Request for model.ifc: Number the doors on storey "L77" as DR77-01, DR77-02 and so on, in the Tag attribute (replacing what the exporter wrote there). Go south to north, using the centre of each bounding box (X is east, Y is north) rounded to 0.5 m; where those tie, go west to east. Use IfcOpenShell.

First a look at what the model holds.

```python
import ifcopenshell
import ifcopenshell.util.element
import ifcopenshell.util.placement

model = ifcopenshell.open("model.ifc")
print(model.schema)
storey = next(s for s in model.by_type("IfcBuildingStorey") if s.Name == "L77")
doors = [e for e in ifcopenshell.util.element.get_decomposition(storey) if e.is_a("IfcDoor")]
for e in sorted(doors, key=lambda e: e.id()):
    origin = ifcopenshell.util.placement.get_local_placement(e.ObjectPlacement)[:3, 3]
    print(e.id(), e.Tag, e.Name, origin.round(2) + 0.0, sep=" | ")
```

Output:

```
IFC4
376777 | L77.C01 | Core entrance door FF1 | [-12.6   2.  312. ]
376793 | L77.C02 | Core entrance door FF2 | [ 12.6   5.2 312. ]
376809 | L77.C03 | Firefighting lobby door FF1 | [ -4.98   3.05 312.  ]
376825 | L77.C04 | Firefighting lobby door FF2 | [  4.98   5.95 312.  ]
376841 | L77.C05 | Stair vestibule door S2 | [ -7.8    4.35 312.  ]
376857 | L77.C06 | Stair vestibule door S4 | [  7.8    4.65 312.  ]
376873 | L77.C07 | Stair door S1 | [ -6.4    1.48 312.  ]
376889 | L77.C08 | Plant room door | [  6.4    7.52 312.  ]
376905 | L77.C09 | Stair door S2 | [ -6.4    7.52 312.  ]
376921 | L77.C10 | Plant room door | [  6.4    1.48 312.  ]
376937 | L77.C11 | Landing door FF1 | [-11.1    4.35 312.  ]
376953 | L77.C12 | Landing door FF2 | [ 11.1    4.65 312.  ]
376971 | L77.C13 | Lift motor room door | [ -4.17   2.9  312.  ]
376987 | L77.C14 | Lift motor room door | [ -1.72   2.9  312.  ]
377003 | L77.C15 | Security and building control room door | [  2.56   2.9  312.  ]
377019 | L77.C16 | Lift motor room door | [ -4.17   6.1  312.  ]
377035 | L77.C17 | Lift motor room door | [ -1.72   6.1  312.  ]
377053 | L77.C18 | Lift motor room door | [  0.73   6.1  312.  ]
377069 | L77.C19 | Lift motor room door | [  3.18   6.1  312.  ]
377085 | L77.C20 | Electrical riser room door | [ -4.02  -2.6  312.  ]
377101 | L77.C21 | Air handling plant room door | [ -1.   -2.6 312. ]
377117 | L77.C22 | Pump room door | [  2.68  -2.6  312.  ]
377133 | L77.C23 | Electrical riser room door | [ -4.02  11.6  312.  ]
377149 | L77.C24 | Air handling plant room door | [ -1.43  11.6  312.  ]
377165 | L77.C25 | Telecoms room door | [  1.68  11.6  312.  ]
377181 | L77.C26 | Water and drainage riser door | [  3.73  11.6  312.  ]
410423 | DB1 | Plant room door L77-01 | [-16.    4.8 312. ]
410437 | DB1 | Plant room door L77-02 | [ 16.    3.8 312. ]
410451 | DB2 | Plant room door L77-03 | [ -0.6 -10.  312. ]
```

```python
import ifcopenshell
import ifcopenshell.geom
import ifcopenshell.util.element
import ifcopenshell.util.shape

model = ifcopenshell.open("model.ifc")
settings = ifcopenshell.geom.settings()
settings.set("use-world-coords", True)


def centre(element):
    shape = ifcopenshell.geom.create_shape(settings, element)
    return ifcopenshell.util.shape.get_bbox_centroid(shape.geometry)


storey = next(s for s in model.by_type("IfcBuildingStorey") if s.Name == "L77")
doors = [e for e in ifcopenshell.util.element.get_decomposition(storey) if e.is_a("IfcDoor")]

# Insertion points can sit at a corner or the storey origin, so sort by the geometry (in metres).
centres = {e: centre(e) for e in doors}
doors.sort(key=lambda e: (round(centres[e][1] / 0.5), centres[e][0]))

for i, e in enumerate(doors, start=1):
    number = f"DR77-{i:02d}"
    e.Tag = number
    print(e.id(), number)

model.write("model_updated.ifc")
```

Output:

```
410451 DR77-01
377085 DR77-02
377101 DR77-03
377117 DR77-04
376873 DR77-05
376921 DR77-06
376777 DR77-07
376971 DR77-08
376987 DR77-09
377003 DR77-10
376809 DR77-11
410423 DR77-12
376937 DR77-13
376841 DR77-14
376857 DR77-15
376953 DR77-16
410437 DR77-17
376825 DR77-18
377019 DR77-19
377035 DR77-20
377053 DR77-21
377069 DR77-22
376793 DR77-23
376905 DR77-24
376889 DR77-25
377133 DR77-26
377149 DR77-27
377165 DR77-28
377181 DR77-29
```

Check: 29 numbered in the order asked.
